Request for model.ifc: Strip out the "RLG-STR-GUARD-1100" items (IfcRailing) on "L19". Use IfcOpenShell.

First a look at what the model holds.

```python
import ifcopenshell
import ifcopenshell.util.element

model = ifcopenshell.open("model.ifc")
print(model.schema)
storey = next(s for s in model.by_type("IfcBuildingStorey") if s.Name == "L19")
railings = [e for e in ifcopenshell.util.element.get_decomposition(storey) if e.is_a("IfcRailing")]
seen = {}
for e in railings:
    element_type = ifcopenshell.util.element.get_type(e)
    name = element_type.Name if element_type not in (None, e) else None
    seen[name] = seen.get(name, 0) + 1
for name, count in sorted(seen.items(), key=str):
    print(count, "x", name)
```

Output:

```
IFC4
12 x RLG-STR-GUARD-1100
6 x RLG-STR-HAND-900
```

```python
import ifcopenshell
import ifcopenshell.api.root
import ifcopenshell.util.element

model = ifcopenshell.open("model.ifc")

storey = next(s for s in model.by_type("IfcBuildingStorey") if s.Name == "L19")
railings = [e for e in ifcopenshell.util.element.get_decomposition(storey) if e.is_a("IfcRailing")]
targets = [e for e in railings if (t := ifcopenshell.util.element.get_type(e)) not in (None, e) and t.Name == "RLG-STR-GUARD-1100"]

for e in targets:
    ifcopenshell.api.root.remove_product(model, product=e)
print(len(targets), "removed")

model.write("model_edited.ifc")
```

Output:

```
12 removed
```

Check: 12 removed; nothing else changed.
